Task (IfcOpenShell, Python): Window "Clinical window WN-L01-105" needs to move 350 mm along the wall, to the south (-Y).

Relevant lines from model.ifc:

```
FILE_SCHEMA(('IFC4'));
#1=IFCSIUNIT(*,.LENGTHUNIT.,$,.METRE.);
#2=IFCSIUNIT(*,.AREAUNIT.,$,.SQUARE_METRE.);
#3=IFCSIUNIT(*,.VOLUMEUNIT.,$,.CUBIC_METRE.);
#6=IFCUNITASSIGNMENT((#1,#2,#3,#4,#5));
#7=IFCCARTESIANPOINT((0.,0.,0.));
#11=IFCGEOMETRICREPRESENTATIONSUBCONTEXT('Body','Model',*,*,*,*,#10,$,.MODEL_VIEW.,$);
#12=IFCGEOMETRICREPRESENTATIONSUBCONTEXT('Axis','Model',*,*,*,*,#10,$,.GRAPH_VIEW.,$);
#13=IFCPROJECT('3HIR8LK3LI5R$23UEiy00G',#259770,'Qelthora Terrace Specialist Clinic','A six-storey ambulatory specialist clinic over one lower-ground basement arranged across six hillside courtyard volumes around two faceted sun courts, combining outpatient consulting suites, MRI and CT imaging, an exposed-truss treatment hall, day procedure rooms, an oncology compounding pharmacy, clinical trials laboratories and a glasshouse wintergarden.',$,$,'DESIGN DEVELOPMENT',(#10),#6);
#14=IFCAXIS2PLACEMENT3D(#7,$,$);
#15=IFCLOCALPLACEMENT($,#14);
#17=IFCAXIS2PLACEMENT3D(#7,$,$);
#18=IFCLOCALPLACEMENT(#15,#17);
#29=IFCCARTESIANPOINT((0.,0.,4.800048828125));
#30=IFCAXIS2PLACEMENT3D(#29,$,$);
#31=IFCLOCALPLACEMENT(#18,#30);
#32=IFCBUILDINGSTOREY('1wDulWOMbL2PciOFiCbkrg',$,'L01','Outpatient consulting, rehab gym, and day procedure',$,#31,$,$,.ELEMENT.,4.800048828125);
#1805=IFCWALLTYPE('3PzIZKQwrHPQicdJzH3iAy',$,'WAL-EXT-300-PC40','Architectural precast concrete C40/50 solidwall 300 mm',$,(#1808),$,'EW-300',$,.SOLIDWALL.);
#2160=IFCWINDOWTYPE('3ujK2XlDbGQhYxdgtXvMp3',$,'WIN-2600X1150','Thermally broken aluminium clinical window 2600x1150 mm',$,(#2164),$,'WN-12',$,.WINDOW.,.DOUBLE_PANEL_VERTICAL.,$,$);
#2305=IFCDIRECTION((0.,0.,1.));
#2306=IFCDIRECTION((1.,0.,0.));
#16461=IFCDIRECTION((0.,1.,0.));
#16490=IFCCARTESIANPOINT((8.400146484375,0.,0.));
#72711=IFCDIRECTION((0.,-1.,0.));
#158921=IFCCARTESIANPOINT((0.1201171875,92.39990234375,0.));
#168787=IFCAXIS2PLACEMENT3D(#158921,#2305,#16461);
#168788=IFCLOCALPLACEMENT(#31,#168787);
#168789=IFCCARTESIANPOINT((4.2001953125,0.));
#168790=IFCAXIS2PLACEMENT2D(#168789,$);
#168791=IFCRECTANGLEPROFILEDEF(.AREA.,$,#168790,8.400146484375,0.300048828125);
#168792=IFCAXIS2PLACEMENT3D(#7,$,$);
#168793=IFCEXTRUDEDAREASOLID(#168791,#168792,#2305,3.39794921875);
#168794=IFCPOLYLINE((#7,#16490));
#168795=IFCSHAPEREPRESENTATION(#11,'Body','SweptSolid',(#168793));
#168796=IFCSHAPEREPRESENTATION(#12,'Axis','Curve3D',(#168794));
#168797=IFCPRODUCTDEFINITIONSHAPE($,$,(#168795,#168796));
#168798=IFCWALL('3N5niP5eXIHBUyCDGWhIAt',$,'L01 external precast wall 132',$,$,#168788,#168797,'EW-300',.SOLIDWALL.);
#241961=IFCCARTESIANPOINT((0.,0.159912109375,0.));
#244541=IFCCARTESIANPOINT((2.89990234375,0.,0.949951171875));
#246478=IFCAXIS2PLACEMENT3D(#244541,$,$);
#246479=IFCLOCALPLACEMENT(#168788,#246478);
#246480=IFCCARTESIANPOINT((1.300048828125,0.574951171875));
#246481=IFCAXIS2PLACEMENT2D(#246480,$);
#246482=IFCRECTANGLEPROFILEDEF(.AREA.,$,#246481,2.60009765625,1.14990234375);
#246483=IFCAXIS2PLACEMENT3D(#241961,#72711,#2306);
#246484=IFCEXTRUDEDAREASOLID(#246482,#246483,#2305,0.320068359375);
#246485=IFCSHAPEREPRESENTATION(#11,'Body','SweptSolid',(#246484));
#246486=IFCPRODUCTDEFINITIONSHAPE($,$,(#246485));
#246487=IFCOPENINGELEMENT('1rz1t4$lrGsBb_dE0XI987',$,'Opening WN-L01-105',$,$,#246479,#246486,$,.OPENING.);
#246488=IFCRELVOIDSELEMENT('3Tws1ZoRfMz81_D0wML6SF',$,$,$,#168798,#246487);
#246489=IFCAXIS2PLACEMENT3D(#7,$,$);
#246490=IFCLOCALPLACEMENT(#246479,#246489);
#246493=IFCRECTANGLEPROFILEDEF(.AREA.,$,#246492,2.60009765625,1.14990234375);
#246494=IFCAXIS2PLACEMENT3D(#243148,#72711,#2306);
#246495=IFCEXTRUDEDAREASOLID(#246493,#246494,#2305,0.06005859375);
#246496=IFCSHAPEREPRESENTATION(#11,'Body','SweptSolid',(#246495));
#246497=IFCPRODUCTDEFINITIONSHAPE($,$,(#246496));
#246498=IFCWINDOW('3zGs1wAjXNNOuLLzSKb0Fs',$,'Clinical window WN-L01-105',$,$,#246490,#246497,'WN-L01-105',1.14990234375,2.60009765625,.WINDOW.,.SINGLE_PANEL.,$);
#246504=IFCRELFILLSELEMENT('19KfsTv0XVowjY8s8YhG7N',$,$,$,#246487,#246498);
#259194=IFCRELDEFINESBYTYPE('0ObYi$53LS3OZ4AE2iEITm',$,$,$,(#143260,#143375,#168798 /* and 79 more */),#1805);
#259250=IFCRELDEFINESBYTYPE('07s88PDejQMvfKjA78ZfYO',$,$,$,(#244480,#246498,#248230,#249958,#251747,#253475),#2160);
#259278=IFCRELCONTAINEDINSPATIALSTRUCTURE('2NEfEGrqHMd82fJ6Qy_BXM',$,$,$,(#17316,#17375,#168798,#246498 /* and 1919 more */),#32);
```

```python
import ifcopenshell
import ifcopenshell.api.geometry
import ifcopenshell.util.placement
import ifcopenshell.util.unit

model = ifcopenshell.open("model.ifc")
unit_scale = ifcopenshell.util.unit.calculate_unit_scale(model)

window = model.by_guid("3zGs1wAjXNNOuLLzSKb0Fs")
opening = window.FillsVoids[0].RelatingOpeningElement
wall = opening.VoidsElements[0].RelatingBuildingElement

wall_matrix = ifcopenshell.util.placement.get_local_placement(wall.ObjectPlacement)
shift = wall_matrix[:3, 0] * -0.35 / unit_scale
before = ifcopenshell.util.placement.get_local_placement(window.ObjectPlacement)[:3, 3].copy()

# The window is placed relative to its opening, so it follows when the opening moves.
matrix = ifcopenshell.util.placement.get_local_placement(opening.ObjectPlacement)
matrix[:3, 3] += shift
ifcopenshell.api.geometry.edit_object_placement(
    model, product=opening, matrix=matrix, is_si=False, should_transform_children=True
)

after = ifcopenshell.util.placement.get_local_placement(window.ObjectPlacement)[:3, 3]
print("window moved by", (after - before).round(3) + 0.0)

model.write("model_v2.ifc")
```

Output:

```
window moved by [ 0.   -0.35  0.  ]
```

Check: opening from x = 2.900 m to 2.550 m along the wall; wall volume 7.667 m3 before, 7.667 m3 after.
